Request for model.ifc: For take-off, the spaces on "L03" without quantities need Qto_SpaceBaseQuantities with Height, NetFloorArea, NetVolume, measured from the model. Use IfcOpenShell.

First a look at what the model holds.

```python
import ifcopenshell
import ifcopenshell.util.element
import ifcopenshell.util.unit

model = ifcopenshell.open("model.ifc")
print(model.schema)
for unit_type in ("LENGTHUNIT", "AREAUNIT", "VOLUMEUNIT"):
    print(unit_type, ifcopenshell.util.unit.calculate_unit_scale(model, unit_type))
storey = next(s for s in model.by_type("IfcBuildingStorey") if s.Name == "L03")
spaces = [e for e in ifcopenshell.util.element.get_decomposition(storey) if e.is_a("IfcSpace")]
for e in sorted(spaces, key=lambda e: e.id()):
    print(e.id(), e.is_a(), e.Name, list(ifcopenshell.util.element.get_psets(e, qtos_only=True)), sep=" | ")
```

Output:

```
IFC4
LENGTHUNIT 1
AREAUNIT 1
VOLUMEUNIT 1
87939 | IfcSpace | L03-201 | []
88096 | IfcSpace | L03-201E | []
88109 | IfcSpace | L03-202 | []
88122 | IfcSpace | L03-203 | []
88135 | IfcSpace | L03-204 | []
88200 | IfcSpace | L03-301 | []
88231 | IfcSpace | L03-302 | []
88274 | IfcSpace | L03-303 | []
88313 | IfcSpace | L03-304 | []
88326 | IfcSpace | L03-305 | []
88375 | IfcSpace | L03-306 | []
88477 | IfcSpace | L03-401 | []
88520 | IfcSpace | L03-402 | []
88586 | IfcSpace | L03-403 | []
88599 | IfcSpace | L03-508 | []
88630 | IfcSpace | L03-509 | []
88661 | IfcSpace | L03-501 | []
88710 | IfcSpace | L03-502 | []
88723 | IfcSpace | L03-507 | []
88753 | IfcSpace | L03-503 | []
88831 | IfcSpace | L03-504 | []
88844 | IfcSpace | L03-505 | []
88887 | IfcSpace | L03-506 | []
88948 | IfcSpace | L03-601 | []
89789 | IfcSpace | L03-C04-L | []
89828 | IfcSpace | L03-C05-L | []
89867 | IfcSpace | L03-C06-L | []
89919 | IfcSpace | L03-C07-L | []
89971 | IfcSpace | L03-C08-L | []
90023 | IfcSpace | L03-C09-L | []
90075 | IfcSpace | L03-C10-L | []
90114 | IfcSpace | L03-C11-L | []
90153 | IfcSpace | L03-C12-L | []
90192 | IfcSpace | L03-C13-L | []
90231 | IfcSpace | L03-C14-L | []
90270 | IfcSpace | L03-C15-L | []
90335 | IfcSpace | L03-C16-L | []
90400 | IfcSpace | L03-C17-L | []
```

```python
import ifcopenshell
import ifcopenshell.api.pset
import ifcopenshell.geom
import ifcopenshell.util.element
import ifcopenshell.util.shape
import ifcopenshell.util.unit

model = ifcopenshell.open("model.ifc")
unit_scale = ifcopenshell.util.unit.calculate_unit_scale(model)
area_scale = ifcopenshell.util.unit.calculate_unit_scale(model, "AREAUNIT")
volume_scale = ifcopenshell.util.unit.calculate_unit_scale(model, "VOLUMEUNIT")
settings = ifcopenshell.geom.settings()

storey = next(s for s in model.by_type("IfcBuildingStorey") if s.Name == "L03")
spaces = [e for e in ifcopenshell.util.element.get_decomposition(storey) if e.is_a("IfcSpace")]

for e in sorted(spaces, key=lambda e: e.id()):
    if ifcopenshell.util.element.get_psets(e, qtos_only=True, should_inherit=False):
        continue
    # Geometry comes back in metres, in the element's own axes.
    shape = ifcopenshell.geom.create_shape(settings, e)
    values = {
        "Height": ifcopenshell.util.shape.get_z(shape.geometry) / unit_scale,
        "NetFloorArea": ifcopenshell.util.shape.get_footprint_area(shape.geometry) / area_scale,
        "NetVolume": ifcopenshell.util.shape.get_volume(shape.geometry) / volume_scale,
    }
    qto = ifcopenshell.api.pset.add_qto(model, product=e, name="Qto_SpaceBaseQuantities")
    ifcopenshell.api.pset.edit_qto(model, qto=qto, properties=values)
    print(e.id(), {k: round(v, 3) for k, v in values.items()})

model.write("model_edited.ifc")
```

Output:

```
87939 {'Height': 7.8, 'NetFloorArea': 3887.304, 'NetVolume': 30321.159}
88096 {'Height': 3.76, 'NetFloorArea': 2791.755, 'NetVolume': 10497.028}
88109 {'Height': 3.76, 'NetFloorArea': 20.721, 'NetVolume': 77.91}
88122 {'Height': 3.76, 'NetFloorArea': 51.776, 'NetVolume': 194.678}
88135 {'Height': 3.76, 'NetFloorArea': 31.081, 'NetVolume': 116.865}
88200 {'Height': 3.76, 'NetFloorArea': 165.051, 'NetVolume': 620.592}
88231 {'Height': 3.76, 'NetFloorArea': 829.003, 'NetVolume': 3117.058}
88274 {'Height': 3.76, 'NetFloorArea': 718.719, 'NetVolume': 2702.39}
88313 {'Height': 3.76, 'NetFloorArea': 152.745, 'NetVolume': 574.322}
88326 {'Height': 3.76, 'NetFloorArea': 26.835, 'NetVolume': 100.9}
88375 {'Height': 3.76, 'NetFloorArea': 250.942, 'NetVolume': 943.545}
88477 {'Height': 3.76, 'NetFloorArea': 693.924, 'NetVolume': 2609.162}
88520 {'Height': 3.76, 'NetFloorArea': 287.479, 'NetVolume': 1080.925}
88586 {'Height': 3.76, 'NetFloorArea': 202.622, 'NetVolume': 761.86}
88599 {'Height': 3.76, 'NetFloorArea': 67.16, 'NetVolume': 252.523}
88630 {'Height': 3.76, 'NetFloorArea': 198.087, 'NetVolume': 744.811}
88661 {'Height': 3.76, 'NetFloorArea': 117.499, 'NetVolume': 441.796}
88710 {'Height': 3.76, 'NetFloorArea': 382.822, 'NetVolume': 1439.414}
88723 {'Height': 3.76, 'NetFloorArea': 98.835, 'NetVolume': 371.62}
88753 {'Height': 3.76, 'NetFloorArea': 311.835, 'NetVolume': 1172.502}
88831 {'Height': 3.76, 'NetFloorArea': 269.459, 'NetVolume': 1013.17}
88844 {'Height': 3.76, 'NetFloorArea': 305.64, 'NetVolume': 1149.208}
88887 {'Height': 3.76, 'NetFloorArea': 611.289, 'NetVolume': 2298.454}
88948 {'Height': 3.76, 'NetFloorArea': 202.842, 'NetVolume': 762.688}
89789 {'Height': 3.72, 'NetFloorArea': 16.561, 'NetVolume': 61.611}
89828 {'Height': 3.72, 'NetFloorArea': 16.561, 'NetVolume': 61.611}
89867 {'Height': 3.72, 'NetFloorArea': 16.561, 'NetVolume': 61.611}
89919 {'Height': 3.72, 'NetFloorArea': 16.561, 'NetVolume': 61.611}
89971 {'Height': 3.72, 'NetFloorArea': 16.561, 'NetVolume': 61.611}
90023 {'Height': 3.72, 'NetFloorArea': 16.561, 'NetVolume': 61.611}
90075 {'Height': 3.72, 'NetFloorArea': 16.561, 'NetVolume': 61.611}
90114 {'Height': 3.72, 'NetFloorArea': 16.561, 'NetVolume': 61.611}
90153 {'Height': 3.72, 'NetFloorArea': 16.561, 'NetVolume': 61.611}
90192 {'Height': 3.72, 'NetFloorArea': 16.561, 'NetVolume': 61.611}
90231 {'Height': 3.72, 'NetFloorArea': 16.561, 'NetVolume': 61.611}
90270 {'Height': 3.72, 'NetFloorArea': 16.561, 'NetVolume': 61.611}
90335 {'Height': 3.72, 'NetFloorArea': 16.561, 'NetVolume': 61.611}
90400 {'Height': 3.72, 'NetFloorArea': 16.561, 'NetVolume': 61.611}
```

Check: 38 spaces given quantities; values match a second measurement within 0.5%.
